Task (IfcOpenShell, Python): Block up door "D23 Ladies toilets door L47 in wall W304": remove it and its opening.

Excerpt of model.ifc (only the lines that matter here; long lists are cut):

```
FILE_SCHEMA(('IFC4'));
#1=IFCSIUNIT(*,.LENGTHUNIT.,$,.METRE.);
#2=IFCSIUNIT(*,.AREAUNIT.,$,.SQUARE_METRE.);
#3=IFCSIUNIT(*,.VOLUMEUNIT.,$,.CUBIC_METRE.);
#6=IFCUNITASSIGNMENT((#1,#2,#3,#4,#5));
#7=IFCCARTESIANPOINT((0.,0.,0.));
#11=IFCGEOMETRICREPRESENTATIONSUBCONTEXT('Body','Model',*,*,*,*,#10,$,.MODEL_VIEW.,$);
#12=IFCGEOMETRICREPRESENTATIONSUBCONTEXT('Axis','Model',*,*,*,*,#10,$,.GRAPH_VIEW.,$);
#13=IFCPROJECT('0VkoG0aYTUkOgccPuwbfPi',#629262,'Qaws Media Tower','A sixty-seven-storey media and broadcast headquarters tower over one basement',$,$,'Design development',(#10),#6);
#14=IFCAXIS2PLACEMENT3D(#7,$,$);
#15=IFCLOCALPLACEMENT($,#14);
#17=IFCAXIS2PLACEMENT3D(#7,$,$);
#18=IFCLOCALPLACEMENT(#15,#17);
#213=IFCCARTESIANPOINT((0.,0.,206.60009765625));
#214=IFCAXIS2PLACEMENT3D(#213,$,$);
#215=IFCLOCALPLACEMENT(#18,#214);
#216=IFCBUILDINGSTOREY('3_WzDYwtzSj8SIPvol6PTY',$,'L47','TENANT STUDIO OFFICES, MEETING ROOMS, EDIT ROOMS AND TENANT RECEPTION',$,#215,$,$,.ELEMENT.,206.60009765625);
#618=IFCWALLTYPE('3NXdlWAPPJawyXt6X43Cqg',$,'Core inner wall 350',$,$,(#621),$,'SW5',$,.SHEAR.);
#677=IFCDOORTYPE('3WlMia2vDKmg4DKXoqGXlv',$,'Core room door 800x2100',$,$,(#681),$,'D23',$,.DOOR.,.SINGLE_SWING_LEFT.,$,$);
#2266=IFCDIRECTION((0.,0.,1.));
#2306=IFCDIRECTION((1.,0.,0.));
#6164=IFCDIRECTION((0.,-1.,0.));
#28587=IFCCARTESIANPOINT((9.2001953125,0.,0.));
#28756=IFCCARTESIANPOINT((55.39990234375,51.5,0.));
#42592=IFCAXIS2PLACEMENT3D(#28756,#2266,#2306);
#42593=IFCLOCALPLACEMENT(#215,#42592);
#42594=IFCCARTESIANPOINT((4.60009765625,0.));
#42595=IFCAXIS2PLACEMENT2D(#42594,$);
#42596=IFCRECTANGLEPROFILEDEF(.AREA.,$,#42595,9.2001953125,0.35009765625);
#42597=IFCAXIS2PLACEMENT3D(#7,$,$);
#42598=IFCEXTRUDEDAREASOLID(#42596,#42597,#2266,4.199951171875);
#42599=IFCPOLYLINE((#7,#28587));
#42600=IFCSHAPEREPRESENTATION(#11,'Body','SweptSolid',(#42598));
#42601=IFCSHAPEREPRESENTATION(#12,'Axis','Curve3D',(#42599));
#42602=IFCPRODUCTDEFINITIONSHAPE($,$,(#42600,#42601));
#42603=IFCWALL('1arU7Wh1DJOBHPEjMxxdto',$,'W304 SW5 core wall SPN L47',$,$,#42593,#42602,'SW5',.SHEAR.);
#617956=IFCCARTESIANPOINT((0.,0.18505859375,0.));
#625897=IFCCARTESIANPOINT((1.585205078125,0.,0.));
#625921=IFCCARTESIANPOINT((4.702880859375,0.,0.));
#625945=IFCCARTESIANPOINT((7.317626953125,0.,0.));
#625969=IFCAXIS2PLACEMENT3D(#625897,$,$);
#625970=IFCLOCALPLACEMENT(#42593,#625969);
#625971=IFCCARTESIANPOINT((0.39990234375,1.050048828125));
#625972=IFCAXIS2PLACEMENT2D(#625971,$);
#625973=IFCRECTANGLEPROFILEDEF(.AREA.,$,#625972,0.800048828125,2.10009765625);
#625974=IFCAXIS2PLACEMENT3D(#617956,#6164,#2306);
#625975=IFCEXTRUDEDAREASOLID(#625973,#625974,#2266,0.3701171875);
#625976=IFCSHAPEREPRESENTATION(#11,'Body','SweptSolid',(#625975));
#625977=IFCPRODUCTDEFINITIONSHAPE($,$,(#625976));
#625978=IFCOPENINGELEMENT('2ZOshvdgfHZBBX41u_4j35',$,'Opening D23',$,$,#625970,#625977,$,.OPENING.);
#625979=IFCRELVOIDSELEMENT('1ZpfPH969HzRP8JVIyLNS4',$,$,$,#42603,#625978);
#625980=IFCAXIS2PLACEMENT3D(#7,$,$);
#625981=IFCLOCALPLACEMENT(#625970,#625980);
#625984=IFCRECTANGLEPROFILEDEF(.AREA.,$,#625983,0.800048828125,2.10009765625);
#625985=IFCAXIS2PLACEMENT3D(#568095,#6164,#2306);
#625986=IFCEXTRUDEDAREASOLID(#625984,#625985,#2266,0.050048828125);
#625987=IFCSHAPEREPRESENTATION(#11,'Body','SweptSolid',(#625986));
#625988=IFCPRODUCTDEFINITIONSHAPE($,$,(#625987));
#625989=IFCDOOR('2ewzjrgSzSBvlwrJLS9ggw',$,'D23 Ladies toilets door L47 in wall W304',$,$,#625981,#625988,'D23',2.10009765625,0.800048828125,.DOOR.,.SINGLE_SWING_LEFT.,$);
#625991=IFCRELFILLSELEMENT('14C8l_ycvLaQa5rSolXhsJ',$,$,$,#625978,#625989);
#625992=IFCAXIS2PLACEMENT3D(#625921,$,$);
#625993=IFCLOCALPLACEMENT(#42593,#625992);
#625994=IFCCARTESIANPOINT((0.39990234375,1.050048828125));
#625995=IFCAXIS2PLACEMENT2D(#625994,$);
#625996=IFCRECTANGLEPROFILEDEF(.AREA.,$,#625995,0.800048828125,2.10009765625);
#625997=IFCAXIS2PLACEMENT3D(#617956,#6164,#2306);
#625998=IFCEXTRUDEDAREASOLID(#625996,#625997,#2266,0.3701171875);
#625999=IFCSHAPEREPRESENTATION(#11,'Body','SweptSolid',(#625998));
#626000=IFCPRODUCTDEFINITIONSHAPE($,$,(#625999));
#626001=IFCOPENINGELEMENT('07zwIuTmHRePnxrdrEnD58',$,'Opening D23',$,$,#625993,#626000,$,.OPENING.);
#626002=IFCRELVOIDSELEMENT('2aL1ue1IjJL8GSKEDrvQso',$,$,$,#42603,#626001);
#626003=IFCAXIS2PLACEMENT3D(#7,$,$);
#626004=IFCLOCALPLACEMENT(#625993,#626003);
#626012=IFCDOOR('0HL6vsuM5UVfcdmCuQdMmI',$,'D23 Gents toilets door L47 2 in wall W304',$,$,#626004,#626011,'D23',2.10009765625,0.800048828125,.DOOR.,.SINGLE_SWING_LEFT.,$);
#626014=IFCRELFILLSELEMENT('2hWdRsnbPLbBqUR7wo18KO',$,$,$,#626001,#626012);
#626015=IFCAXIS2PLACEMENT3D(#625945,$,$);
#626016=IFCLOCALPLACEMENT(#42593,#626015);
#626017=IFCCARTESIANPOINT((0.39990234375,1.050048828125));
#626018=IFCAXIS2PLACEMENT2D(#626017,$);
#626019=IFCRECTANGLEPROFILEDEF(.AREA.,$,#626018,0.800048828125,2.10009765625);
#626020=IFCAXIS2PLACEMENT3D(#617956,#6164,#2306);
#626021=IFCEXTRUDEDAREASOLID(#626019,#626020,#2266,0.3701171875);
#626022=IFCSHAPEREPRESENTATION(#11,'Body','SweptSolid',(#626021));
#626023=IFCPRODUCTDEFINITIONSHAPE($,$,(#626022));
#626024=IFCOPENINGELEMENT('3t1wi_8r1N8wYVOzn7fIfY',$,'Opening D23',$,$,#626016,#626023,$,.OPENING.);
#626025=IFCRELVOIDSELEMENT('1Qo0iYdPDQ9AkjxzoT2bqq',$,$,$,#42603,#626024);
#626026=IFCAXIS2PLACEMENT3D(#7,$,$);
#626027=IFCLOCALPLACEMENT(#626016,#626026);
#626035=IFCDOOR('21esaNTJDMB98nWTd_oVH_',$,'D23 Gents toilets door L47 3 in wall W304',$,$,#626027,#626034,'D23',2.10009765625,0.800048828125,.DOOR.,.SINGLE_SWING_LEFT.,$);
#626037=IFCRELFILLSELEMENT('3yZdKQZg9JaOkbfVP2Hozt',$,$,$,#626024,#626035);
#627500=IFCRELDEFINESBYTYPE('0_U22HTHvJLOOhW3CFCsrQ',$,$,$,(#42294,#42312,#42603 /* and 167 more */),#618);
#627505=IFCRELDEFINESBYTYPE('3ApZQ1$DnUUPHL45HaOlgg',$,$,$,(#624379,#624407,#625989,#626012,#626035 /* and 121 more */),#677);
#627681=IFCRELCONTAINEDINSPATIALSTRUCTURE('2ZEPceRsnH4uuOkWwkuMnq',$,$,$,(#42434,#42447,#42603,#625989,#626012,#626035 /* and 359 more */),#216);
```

```python
import ifcopenshell
import ifcopenshell.api.feature
import ifcopenshell.api.root
import ifcopenshell.geom
import ifcopenshell.util.shape

model = ifcopenshell.open("model.ifc")
settings = ifcopenshell.geom.settings()


def volume(element):
    """Net volume in cubic metres, openings subtracted."""
    shape = ifcopenshell.geom.create_shape(settings, element)
    return ifcopenshell.util.shape.get_volume(shape.geometry)


door = model.by_guid("2ewzjrgSzSBvlwrJLS9ggw")
opening = door.FillsVoids[0].RelatingOpeningElement
wall = opening.VoidsElements[0].RelatingBuildingElement
before = volume(wall)

ifcopenshell.api.root.remove_product(model, product=door)
ifcopenshell.api.feature.remove_feature(model, feature=opening)

after = volume(wall)

print(f"wall volume {before:.3f} -> {after:.3f} m3")

model.write("model_updated.ifc")
```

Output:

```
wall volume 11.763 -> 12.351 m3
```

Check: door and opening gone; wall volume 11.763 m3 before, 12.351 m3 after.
